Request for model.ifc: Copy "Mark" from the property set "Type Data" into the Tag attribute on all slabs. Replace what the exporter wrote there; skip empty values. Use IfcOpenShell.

First a look at what the model holds.

```python
import ifcopenshell
import ifcopenshell.util.element

model = ifcopenshell.open("model.ifc")
print(model.schema)
slabs = model.by_type("IfcSlab")
print(len(slabs), "slabs")
for e in slabs[:8]:
    source = ifcopenshell.util.element.get_pset(e, "Type Data", "Mark")
    target = e.Tag
    print(e.id(), repr(source), repr(target), sep=" | ")
```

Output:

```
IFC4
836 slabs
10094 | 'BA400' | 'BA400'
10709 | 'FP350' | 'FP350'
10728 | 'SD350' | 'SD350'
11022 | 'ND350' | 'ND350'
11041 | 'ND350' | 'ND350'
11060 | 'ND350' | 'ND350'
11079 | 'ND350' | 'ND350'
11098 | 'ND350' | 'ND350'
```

```python
import ifcopenshell
import ifcopenshell.util.element

model = ifcopenshell.open("model.ifc")

count = 0
for e in model.by_type("IfcSlab"):
    value = ifcopenshell.util.element.get_pset(e, "Type Data", "Mark")
    current = e.Tag
    if not value or not value.strip() or current == value:
        continue
    e.Tag = value
    count += 1

print(count, "slabs updated")

model.write("model_v2.ifc")
```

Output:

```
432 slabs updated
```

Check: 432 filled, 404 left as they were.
